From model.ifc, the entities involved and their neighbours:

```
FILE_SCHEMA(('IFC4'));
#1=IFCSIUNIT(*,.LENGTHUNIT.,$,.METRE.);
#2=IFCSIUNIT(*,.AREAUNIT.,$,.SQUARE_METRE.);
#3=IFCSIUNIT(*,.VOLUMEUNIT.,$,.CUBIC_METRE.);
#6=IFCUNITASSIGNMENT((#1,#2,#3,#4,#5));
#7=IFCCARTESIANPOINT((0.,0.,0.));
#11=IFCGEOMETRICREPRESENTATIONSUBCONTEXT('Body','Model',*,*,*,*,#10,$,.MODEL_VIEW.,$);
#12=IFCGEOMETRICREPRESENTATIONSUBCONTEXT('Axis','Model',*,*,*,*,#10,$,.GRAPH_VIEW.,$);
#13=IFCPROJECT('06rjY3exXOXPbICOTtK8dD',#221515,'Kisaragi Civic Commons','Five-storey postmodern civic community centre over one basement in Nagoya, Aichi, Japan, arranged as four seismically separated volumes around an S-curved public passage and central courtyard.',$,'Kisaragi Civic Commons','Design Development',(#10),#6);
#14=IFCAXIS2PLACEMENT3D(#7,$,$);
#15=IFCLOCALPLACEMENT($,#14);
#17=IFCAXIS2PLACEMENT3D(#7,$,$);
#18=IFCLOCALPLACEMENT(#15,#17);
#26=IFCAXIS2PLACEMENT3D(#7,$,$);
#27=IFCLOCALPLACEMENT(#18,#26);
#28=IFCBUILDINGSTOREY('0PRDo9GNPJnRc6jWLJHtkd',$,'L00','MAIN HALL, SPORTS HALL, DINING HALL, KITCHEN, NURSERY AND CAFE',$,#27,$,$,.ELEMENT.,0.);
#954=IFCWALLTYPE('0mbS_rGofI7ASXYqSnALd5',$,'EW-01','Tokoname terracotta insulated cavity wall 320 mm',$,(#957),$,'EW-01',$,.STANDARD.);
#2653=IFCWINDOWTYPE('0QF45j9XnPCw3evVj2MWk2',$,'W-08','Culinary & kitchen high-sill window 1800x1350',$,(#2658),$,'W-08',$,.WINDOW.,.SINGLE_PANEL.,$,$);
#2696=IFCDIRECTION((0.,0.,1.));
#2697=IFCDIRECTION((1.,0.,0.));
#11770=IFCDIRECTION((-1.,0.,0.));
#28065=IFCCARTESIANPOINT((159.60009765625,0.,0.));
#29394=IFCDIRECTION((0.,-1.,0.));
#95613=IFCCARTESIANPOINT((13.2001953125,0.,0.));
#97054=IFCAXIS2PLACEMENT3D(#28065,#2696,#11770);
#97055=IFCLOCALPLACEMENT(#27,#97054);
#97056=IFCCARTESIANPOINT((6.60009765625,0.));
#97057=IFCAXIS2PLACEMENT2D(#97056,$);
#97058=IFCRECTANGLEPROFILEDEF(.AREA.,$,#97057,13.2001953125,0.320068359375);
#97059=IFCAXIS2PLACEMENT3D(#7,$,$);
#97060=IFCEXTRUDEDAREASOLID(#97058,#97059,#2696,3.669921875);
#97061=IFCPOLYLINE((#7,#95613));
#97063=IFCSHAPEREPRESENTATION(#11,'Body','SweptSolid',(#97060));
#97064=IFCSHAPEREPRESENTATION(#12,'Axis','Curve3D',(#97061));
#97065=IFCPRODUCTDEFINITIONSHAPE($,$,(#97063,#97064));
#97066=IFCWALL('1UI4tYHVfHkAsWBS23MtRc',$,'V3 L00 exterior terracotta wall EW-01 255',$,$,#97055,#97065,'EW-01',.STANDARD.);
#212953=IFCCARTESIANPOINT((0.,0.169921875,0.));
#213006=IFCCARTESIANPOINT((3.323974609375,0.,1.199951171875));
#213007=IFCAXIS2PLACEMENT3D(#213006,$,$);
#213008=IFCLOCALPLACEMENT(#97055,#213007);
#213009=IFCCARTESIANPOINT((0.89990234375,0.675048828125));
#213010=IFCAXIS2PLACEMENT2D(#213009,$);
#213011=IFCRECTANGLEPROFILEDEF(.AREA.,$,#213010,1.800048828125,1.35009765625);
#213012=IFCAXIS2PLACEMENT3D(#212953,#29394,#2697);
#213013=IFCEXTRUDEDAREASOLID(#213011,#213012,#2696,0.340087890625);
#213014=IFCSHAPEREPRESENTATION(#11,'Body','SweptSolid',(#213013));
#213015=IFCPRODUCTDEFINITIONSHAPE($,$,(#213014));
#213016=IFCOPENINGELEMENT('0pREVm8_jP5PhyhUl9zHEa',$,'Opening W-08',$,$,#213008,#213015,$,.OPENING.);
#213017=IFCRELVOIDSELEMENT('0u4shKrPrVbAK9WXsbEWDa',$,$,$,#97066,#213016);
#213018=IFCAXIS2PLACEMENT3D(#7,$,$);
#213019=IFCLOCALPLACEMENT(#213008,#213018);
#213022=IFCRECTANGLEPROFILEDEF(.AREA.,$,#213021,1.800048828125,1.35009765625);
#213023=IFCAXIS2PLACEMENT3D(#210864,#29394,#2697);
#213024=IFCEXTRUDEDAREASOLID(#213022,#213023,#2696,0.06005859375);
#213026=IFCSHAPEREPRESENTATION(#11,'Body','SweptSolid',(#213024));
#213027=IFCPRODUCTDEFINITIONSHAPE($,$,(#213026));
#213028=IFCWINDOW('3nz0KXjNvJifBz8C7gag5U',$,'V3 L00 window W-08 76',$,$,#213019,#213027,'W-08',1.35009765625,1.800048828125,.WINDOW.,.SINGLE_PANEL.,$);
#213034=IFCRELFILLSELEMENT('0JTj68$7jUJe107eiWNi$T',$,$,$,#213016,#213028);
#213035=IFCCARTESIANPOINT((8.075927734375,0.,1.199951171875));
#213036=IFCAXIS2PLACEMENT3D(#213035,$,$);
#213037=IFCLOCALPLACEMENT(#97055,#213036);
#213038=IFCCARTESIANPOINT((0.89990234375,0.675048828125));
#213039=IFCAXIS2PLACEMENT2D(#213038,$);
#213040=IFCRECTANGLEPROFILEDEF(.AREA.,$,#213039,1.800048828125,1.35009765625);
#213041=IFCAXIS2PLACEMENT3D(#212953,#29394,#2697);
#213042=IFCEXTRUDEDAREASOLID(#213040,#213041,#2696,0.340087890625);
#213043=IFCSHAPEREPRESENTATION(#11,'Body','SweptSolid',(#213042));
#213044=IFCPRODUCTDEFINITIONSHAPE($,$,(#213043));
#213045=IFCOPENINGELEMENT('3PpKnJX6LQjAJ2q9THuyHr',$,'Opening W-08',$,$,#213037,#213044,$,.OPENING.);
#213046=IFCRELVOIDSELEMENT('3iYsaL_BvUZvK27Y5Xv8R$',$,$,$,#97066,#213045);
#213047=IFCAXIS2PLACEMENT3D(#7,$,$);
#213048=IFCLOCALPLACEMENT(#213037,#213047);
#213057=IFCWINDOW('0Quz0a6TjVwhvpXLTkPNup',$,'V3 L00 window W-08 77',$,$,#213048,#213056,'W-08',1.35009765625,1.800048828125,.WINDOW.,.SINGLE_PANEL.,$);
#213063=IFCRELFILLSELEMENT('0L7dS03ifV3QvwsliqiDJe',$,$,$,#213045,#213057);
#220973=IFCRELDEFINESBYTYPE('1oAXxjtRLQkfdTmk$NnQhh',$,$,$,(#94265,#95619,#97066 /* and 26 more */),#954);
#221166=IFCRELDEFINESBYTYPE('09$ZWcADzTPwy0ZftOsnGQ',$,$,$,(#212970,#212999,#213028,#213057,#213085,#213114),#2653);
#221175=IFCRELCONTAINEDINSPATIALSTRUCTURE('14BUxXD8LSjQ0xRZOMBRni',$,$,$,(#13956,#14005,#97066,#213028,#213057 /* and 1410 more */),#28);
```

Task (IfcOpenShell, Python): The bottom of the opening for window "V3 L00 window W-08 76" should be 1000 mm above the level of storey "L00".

```python
import numpy as np
import ifcopenshell
import ifcopenshell.api.geometry
import ifcopenshell.geom
import ifcopenshell.util.element
import ifcopenshell.util.placement
import ifcopenshell.util.shape
import ifcopenshell.util.unit

model = ifcopenshell.open("model.ifc")
unit_scale = ifcopenshell.util.unit.calculate_unit_scale(model)

window = model.by_guid("3nz0KXjNvJifBz8C7gag5U")
opening = window.FillsVoids[0].RelatingOpeningElement
storey = ifcopenshell.util.element.get_container(window, ifc_class="IfcBuildingStorey")
level = ifcopenshell.util.placement.get_local_placement(storey.ObjectPlacement)[2, 3]

# The opening's origin need not be at the sill, so measure its lowest point.
shape = ifcopenshell.geom.create_shape(ifcopenshell.geom.settings(), opening)
bottom = ifcopenshell.util.shape.get_shape_bottom_elevation(shape, shape.geometry) / unit_scale
dz = level + 1.0 - bottom

shift = np.array([0.0, 0.0, dz])
# The window is placed relative to its opening, so it follows when the opening moves.
matrix = ifcopenshell.util.placement.get_local_placement(opening.ObjectPlacement)
matrix[:3, 3] += shift
ifcopenshell.api.geometry.edit_object_placement(
    model, product=opening, matrix=matrix, is_si=False, should_transform_children=True
)

print(f"moved by {dz * unit_scale:+.3f} m")

model.write("model_updated.ifc")
```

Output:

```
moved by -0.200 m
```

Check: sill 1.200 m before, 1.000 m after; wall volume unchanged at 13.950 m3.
